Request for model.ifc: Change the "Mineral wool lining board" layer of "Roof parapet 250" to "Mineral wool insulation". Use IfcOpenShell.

First a look at what the model holds.

```python
import ifcopenshell
import ifcopenshell.util.element

model = ifcopenshell.open("model.ifc")
print(model.schema)
for layer_set in model.by_type("IfcMaterialLayerSet"):
    if layer_set.LayerSetName == "Roof parapet 250":
        for layer in layer_set.MaterialLayers:
            print(layer.id(), layer.Material and layer.Material.Name, layer.LayerThickness, sep=" | ")
        print(len(ifcopenshell.util.element.get_elements_by_material(model, layer_set)), "elements and types use it")
print(sorted(m.Name for m in model.by_type("IfcMaterial") if m.Name)[:60])
```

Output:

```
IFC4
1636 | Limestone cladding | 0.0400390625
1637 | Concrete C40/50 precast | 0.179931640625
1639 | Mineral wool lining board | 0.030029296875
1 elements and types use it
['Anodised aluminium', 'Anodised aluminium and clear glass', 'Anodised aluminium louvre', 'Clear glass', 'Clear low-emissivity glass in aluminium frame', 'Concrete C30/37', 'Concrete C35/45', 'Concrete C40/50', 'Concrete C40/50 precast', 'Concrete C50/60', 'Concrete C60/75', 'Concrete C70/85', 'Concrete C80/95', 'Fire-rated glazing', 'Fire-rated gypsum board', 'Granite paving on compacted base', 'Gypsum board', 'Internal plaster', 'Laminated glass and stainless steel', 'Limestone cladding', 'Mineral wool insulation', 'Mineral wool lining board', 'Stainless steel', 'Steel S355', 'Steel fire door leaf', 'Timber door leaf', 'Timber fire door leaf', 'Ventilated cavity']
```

```python
import ifcopenshell
import ifcopenshell.api.material

model = ifcopenshell.open("model.ifc")

layer_set = next(s for s in model.by_type("IfcMaterialLayerSet") if s.LayerSetName == "Roof parapet 250")
layer = next(l for l in layer_set.MaterialLayers if l.Material and l.Material.Name == "Mineral wool lining board")
material = next(m for m in model.by_type("IfcMaterial") if m.Name == "Mineral wool insulation")

# Point this one layer at the other material; renaming the old one would change it everywhere.
ifcopenshell.api.material.edit_layer(model, layer=layer, attributes={}, material=material)

print([l.Material.Name if l.Material else None for l in layer_set.MaterialLayers])

model.write("model_rev.ifc")
```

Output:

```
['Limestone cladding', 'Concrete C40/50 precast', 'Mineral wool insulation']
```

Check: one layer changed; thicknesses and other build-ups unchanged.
